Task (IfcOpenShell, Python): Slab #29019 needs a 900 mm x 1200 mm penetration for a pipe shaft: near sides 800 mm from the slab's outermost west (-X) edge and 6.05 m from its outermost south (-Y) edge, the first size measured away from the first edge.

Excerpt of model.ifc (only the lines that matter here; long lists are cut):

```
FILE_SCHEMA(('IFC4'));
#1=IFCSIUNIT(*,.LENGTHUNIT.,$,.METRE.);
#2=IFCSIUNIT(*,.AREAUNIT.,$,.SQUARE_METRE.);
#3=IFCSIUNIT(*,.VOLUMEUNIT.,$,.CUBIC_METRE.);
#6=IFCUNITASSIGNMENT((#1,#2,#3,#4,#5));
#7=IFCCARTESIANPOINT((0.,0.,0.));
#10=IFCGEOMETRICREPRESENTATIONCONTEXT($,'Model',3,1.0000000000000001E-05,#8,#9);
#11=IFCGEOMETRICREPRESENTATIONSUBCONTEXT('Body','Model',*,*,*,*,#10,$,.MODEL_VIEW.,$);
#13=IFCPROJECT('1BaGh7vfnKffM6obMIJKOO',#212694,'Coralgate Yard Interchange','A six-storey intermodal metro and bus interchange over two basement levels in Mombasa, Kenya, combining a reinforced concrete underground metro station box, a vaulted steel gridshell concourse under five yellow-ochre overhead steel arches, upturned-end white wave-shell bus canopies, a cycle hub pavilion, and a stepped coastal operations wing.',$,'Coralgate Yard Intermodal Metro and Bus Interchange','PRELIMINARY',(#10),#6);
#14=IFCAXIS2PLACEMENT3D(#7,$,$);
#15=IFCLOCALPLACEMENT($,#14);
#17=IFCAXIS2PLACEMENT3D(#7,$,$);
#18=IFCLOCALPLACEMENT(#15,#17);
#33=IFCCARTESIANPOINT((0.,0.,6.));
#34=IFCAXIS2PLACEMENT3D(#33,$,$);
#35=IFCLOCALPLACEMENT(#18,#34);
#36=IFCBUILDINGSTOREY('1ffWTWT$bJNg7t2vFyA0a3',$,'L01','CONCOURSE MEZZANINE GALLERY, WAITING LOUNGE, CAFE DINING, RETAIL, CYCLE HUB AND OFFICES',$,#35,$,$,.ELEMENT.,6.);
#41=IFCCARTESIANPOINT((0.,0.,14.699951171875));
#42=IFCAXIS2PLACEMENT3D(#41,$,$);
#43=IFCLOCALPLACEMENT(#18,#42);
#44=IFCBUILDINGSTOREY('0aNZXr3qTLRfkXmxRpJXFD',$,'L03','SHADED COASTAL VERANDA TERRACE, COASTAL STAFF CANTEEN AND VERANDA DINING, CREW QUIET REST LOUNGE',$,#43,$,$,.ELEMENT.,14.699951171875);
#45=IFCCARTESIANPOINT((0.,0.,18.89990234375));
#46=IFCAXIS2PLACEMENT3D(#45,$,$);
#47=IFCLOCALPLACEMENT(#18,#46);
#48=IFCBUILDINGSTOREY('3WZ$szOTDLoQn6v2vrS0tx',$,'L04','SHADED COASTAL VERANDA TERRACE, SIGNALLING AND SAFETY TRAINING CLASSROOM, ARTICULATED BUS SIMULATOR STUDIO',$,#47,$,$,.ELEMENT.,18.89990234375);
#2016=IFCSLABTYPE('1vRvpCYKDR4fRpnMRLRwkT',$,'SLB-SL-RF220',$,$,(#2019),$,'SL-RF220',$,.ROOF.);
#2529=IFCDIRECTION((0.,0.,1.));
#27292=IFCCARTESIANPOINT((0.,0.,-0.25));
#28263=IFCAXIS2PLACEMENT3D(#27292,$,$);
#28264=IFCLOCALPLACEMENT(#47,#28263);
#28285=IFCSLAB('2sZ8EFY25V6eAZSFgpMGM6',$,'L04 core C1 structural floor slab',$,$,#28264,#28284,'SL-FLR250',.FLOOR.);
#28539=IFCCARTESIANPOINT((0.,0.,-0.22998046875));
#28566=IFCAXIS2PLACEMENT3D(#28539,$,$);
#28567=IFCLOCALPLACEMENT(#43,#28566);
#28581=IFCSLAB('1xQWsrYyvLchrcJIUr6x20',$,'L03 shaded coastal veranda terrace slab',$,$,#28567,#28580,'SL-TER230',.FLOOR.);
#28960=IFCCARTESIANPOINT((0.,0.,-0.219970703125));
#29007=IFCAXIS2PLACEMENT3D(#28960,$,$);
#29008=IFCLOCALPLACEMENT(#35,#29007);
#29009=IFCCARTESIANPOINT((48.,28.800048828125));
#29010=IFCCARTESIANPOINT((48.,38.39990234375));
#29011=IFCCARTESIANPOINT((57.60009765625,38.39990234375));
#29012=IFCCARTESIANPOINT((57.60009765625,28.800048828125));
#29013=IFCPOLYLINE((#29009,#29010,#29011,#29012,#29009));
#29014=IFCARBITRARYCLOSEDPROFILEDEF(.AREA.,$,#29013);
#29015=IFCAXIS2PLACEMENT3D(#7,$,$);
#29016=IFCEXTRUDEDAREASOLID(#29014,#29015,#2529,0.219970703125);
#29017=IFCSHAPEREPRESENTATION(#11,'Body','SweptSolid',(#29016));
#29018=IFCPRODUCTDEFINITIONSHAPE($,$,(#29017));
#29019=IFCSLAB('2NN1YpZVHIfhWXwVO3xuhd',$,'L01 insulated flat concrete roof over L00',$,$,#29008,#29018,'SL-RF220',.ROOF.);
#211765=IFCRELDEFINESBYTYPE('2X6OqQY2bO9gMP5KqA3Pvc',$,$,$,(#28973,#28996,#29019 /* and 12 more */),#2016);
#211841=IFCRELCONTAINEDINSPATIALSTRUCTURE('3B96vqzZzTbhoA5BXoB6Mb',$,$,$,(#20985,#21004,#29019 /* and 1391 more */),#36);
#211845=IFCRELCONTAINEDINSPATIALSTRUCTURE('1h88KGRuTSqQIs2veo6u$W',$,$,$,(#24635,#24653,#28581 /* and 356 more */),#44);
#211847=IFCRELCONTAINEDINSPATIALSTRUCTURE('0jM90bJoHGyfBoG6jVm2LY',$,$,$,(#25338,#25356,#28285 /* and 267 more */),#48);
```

```python
import numpy as np
import ifcopenshell
import ifcopenshell.api.feature
import ifcopenshell.api.geometry
import ifcopenshell.api.root
import ifcopenshell.geom
import ifcopenshell.util.placement
import ifcopenshell.util.representation
import ifcopenshell.util.shape
import ifcopenshell.util.unit

model = ifcopenshell.open("model.ifc")
unit_scale = ifcopenshell.util.unit.calculate_unit_scale(model)
settings = ifcopenshell.geom.settings()


def volume(element):
    """Net volume in cubic metres, openings subtracted."""
    shape = ifcopenshell.geom.create_shape(settings, element)
    return ifcopenshell.util.shape.get_volume(shape.geometry)


slab = model.by_id(29019)
before = volume(slab)

# Extent in the slab's own axes, in metres. The edges named are its -X and -Y sides.
slab_shape = ifcopenshell.geom.create_shape(settings, slab)
vertices = ifcopenshell.util.shape.get_vertices(slab_shape.geometry)
x_min, y_min, bottom = vertices.min(axis=0)
top = vertices[:, 2].max()

opening = ifcopenshell.api.root.create_entity(model, ifc_class="IfcOpeningElement", name="Pipe shaft opening", predefined_type="OPENING")
context = ifcopenshell.util.representation.get_context(model, "Model", "Body", "MODEL_VIEW")
width, depth = 0.9, 1.2
outline = [(0.0, 0.0), (width, 0.0), (width, depth), (0.0, depth), (0.0, 0.0)]
# Overshoot both faces by 50 mm so the cut is clean.
shape = ifcopenshell.api.geometry.add_slab_representation(
    model, context=context, depth=top - bottom + 0.1, polyline=outline
)
ifcopenshell.api.geometry.assign_representation(model, product=opening, representation=shape)

matrix = ifcopenshell.util.placement.get_local_placement(slab.ObjectPlacement)
matrix[:, 3] = matrix @ np.append(np.array([x_min + 0.8, y_min + 6.05, bottom - 0.05]) / unit_scale, 1.0)
ifcopenshell.api.geometry.edit_object_placement(model, product=opening, matrix=matrix, is_si=False)
ifcopenshell.api.feature.add_feature(model, feature=opening, element=slab)

after = volume(slab)

print(f"slab volume {before:.3f} -> {after:.3f} m3")

model.write("model_rev.ifc")
```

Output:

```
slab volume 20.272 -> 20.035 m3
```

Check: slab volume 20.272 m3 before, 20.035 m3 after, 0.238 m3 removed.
